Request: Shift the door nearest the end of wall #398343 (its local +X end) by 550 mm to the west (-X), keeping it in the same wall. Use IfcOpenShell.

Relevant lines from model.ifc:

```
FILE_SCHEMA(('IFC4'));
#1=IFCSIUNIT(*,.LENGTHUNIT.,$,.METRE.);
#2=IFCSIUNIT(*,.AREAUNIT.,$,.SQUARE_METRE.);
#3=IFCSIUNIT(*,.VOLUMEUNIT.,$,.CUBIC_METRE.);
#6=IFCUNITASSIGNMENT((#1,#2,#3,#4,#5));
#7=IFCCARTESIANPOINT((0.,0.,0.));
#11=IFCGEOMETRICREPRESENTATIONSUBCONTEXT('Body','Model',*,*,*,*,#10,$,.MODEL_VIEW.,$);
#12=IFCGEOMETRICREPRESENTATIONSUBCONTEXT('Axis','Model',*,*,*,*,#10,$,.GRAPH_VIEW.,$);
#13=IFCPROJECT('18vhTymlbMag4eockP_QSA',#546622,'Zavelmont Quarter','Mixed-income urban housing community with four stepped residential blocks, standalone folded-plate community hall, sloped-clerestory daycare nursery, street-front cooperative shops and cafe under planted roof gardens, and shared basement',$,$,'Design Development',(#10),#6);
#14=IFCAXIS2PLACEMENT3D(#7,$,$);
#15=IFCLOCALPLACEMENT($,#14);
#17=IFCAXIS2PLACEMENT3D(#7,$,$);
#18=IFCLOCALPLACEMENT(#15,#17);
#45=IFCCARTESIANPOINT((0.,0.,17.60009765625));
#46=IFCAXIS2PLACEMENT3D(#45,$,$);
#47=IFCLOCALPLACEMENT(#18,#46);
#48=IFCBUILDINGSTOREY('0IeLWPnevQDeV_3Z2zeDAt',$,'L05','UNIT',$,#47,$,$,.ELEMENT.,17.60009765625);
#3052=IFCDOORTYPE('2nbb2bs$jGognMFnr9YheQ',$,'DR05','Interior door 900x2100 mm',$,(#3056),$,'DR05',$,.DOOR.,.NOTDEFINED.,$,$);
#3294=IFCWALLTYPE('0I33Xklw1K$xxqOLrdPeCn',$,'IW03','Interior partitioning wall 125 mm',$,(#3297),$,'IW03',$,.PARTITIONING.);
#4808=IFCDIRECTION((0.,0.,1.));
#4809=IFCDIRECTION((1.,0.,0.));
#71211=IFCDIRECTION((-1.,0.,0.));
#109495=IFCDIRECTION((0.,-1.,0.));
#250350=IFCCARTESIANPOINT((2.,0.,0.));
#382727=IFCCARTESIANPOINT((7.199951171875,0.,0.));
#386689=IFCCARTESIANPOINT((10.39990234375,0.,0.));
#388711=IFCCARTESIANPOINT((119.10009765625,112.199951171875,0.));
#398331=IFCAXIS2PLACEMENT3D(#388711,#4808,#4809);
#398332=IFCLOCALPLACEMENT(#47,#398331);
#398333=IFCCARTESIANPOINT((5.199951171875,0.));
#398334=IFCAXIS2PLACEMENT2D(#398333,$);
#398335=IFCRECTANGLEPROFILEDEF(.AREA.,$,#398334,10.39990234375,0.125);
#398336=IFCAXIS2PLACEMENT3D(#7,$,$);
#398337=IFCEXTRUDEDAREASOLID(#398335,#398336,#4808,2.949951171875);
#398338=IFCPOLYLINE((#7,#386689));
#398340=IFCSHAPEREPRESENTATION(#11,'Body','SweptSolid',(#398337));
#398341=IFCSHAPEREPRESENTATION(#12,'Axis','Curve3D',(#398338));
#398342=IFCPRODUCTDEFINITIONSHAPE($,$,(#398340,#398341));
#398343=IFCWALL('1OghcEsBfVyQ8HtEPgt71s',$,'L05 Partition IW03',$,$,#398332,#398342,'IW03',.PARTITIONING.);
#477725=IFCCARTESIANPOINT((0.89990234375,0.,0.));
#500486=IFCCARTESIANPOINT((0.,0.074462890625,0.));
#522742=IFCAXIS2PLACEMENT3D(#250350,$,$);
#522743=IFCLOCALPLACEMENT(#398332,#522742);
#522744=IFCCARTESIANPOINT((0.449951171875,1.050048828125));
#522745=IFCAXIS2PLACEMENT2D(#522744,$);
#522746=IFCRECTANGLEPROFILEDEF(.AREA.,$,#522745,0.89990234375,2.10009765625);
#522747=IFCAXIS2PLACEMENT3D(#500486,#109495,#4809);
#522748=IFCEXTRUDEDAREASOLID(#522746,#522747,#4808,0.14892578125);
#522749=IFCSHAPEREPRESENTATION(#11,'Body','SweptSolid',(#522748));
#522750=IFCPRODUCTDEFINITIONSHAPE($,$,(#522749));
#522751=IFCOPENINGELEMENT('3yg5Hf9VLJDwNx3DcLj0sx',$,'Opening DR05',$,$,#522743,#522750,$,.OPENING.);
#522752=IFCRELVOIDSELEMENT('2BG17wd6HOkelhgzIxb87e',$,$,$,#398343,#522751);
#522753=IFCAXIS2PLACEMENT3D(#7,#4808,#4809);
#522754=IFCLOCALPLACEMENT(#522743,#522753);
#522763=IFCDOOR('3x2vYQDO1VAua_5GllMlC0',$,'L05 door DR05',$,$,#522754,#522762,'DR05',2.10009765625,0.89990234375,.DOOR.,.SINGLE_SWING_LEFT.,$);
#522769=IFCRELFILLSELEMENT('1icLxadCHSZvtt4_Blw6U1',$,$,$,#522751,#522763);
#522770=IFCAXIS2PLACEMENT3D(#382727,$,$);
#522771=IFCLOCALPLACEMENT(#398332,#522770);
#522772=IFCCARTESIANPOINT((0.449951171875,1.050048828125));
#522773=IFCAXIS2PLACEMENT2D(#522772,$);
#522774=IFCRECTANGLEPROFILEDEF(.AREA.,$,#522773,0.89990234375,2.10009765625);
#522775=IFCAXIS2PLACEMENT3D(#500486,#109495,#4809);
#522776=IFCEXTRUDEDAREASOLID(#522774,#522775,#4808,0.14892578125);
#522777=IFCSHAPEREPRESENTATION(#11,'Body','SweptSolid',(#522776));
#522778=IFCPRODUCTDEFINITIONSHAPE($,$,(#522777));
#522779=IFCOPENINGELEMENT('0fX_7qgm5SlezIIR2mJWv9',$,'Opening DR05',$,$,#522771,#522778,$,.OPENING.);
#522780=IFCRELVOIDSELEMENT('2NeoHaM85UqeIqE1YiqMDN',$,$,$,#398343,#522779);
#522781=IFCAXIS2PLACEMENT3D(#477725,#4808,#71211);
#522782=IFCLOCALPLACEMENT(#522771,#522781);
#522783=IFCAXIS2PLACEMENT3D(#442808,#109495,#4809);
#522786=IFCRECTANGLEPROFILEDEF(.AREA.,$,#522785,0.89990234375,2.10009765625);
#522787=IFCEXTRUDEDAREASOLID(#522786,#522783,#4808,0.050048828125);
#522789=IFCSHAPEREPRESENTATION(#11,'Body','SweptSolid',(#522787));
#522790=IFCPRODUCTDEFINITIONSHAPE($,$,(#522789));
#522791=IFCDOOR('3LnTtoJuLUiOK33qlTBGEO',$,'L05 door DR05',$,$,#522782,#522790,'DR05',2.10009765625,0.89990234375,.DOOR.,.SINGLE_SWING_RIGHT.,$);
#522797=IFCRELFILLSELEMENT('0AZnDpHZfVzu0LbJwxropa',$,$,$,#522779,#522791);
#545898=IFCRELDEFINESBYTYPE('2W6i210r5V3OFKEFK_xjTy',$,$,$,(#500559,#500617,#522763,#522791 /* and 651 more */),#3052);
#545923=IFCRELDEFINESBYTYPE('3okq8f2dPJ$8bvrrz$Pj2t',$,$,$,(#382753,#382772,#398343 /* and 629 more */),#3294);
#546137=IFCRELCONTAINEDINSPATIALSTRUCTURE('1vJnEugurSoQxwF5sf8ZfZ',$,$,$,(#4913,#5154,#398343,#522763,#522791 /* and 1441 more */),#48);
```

```python
import ifcopenshell
import ifcopenshell.api.geometry
import ifcopenshell.util.placement

model = ifcopenshell.open("model.ifc")

door = model.by_id(522791)
opening = door.FillsVoids[0].RelatingOpeningElement
wall = opening.VoidsElements[0].RelatingBuildingElement

wall_matrix = ifcopenshell.util.placement.get_local_placement(wall.ObjectPlacement)
shift = wall_matrix[:3, 0] * -0.55
before = ifcopenshell.util.placement.get_local_placement(door.ObjectPlacement)[:3, 3].copy()

# The door is placed relative to its opening, so it follows when the opening moves.
matrix = ifcopenshell.util.placement.get_local_placement(opening.ObjectPlacement)
matrix[:3, 3] += shift
ifcopenshell.api.geometry.edit_object_placement(
    model, product=opening, matrix=matrix, is_si=False, should_transform_children=True
)

after = ifcopenshell.util.placement.get_local_placement(door.ObjectPlacement)[:3, 3]
print("door moved by", (after - before).round(3) + 0.0)

model.write("model_v2.ifc")
```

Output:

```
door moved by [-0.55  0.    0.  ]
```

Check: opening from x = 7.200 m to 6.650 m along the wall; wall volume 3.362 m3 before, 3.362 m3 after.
